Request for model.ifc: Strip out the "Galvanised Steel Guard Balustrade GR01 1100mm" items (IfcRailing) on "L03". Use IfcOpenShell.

First a look at what the model holds.

```python
import ifcopenshell
import ifcopenshell.util.element

model = ifcopenshell.open("model.ifc")
print(model.schema)
storey = next(s for s in model.by_type("IfcBuildingStorey") if s.Name == "L03")
railings = [e for e in ifcopenshell.util.element.get_decomposition(storey) if e.is_a("IfcRailing")]
seen = {}
for e in railings:
    element_type = ifcopenshell.util.element.get_type(e)
    name = element_type.Name if element_type not in (None, e) else None
    seen[name] = seen.get(name, 0) + 1
for name, count in sorted(seen.items(), key=str):
    print(count, "x", name)
```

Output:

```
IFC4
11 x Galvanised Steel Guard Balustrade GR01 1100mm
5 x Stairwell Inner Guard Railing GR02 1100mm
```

```python
import ifcopenshell
import ifcopenshell.api.root
import ifcopenshell.util.element

model = ifcopenshell.open("model.ifc")

storey = next(s for s in model.by_type("IfcBuildingStorey") if s.Name == "L03")
railings = [e for e in ifcopenshell.util.element.get_decomposition(storey) if e.is_a("IfcRailing")]
targets = [e for e in railings if (t := ifcopenshell.util.element.get_type(e)) not in (None, e) and t.Name == "Galvanised Steel Guard Balustrade GR01 1100mm"]

for e in targets:
    ifcopenshell.api.root.remove_product(model, product=e)
print(len(targets), "removed")

model.write("model_edited.ifc")
```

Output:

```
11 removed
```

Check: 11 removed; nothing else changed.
